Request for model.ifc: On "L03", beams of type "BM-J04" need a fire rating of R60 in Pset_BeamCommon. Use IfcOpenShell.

First a look at what the model holds.

```python
import ifcopenshell
import ifcopenshell.util.element

model = ifcopenshell.open("model.ifc")
print(model.schema)
storey = next(s for s in model.by_type("IfcBuildingStorey") if s.Name == "L03")
beams = [e for e in ifcopenshell.util.element.get_decomposition(storey) if e.is_a("IfcBeam")]
seen = {}
for e in beams:
    element_type = ifcopenshell.util.element.get_type(e)
    key = (element_type.Name if element_type != e and element_type else None, ifcopenshell.util.element.get_pset(e, "Pset_BeamCommon", "FireRating"))
    seen[key] = seen.get(key, 0) + 1
for (name, value), count in sorted(seen.items(), key=str):
    print(count, "x", name, "|", value)
```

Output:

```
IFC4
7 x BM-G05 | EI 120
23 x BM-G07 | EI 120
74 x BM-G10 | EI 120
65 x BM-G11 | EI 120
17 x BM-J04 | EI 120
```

```python
import ifcopenshell
import ifcopenshell.api.pset
import ifcopenshell.util.element

model = ifcopenshell.open("model.ifc")

storey = next(s for s in model.by_type("IfcBuildingStorey") if s.Name == "L03")
beams = [e for e in ifcopenshell.util.element.get_decomposition(storey) if e.is_a("IfcBeam")]

count = 0
for e in beams:
    element_type = ifcopenshell.util.element.get_type(e)
    if element_type in (None, e) or element_type.Name != "BM-J04":
        continue
    # add_pset returns the element's existing set when there is one.
    pset = ifcopenshell.api.pset.add_pset(model, product=e, name="Pset_BeamCommon")
    ifcopenshell.api.pset.edit_pset(model, pset=pset, properties={"FireRating": "R60"})
    count += 1

print(count, "beams updated")

model.write("model-out.ifc")
```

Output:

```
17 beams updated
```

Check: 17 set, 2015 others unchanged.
